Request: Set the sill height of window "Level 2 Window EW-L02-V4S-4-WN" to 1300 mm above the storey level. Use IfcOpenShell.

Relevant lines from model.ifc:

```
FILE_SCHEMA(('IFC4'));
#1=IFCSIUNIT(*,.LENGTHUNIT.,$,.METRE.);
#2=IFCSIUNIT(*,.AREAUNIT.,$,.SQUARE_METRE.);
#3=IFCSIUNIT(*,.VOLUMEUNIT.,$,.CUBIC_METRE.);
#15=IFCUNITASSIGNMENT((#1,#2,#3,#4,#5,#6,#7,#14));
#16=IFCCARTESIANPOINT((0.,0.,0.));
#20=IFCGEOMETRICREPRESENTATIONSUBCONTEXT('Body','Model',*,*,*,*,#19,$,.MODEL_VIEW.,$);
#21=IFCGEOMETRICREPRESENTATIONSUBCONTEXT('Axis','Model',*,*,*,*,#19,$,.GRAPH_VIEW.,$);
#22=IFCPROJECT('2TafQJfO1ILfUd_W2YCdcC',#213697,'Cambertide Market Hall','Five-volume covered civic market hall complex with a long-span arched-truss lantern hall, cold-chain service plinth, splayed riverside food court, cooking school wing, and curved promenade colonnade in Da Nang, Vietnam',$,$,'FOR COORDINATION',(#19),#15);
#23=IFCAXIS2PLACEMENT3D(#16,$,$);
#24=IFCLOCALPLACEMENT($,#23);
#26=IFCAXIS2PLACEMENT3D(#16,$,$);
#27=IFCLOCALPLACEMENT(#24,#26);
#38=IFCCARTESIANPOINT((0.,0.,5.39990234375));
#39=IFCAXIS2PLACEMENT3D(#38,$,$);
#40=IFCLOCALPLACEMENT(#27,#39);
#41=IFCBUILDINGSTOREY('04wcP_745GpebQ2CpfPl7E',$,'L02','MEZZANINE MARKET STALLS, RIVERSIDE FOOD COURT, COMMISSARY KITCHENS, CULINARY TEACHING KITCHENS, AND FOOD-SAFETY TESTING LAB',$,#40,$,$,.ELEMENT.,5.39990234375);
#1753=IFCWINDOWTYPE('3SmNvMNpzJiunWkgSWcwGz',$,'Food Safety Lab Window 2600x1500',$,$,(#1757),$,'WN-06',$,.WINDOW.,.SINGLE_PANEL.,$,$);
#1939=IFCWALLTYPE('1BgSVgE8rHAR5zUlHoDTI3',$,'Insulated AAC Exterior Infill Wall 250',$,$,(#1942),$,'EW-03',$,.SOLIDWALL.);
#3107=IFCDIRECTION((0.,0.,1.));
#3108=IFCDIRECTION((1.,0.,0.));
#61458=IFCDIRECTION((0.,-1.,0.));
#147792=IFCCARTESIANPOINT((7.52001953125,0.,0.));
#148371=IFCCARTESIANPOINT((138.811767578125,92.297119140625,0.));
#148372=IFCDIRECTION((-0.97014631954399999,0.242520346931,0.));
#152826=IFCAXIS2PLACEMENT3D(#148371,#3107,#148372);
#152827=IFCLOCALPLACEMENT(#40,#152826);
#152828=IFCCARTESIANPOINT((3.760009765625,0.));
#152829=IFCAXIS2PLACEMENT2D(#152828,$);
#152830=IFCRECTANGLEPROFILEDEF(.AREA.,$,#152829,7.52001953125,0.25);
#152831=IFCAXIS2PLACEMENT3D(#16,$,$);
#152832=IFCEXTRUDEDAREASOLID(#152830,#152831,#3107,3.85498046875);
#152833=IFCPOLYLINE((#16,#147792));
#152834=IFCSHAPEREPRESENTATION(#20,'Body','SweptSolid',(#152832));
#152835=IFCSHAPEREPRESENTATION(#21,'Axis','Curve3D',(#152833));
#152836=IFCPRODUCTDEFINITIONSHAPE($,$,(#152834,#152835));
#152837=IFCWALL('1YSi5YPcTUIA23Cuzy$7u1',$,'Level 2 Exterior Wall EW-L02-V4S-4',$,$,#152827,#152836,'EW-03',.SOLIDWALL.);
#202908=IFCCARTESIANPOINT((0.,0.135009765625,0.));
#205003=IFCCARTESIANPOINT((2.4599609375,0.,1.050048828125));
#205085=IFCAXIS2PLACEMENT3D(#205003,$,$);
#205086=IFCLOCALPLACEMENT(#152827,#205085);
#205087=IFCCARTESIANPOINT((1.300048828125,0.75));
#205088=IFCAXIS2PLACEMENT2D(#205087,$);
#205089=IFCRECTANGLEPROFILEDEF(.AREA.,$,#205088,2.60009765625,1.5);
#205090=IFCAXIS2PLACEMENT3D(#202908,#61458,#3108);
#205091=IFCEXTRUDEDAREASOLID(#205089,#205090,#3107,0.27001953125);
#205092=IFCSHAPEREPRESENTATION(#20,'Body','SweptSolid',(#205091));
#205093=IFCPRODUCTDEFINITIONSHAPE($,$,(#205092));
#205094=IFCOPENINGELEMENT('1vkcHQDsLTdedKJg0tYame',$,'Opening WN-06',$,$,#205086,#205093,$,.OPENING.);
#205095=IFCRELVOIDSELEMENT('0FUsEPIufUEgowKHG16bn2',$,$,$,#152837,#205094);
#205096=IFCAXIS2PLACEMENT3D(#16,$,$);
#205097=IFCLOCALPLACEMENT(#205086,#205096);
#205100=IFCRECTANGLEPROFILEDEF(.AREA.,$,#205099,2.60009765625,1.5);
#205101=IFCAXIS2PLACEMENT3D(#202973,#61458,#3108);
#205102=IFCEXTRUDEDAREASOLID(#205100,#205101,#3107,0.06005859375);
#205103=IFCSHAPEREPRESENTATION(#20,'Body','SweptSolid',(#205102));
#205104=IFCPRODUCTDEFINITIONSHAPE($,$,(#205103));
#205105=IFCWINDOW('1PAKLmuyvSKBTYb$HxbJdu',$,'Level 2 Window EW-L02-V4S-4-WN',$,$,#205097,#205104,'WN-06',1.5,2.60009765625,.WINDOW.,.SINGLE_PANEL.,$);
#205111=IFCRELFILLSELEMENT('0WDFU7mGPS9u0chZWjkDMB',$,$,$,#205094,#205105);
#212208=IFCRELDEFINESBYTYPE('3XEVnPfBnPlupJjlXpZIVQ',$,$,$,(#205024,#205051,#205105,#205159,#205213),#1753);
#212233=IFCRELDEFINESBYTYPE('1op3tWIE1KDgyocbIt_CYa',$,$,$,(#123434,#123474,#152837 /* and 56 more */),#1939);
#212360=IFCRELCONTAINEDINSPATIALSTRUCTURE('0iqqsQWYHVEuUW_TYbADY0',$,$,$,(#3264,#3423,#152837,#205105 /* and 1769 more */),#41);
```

```python
import numpy as np
import ifcopenshell
import ifcopenshell.api.geometry
import ifcopenshell.geom
import ifcopenshell.util.element
import ifcopenshell.util.placement
import ifcopenshell.util.shape
import ifcopenshell.util.unit

model = ifcopenshell.open("model.ifc")
unit_scale = ifcopenshell.util.unit.calculate_unit_scale(model)

window = model.by_guid("1PAKLmuyvSKBTYb$HxbJdu")
opening = window.FillsVoids[0].RelatingOpeningElement
storey = ifcopenshell.util.element.get_container(window, ifc_class="IfcBuildingStorey")
level = ifcopenshell.util.placement.get_local_placement(storey.ObjectPlacement)[2, 3]

# The opening's origin need not be at the sill, so measure its lowest point.
shape = ifcopenshell.geom.create_shape(ifcopenshell.geom.settings(), opening)
bottom = ifcopenshell.util.shape.get_shape_bottom_elevation(shape, shape.geometry) / unit_scale
dz = level + 1.3 / unit_scale - bottom

shift = np.array([0.0, 0.0, dz])
# The window is placed relative to its opening, so it follows when the opening moves.
matrix = ifcopenshell.util.placement.get_local_placement(opening.ObjectPlacement)
matrix[:3, 3] += shift
ifcopenshell.api.geometry.edit_object_placement(
    model, product=opening, matrix=matrix, is_si=False, should_transform_children=True
)

print(f"moved by {dz * unit_scale:+.3f} m")

model.write("model_edited.ifc")
```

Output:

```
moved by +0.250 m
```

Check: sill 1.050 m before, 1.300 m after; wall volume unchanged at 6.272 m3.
